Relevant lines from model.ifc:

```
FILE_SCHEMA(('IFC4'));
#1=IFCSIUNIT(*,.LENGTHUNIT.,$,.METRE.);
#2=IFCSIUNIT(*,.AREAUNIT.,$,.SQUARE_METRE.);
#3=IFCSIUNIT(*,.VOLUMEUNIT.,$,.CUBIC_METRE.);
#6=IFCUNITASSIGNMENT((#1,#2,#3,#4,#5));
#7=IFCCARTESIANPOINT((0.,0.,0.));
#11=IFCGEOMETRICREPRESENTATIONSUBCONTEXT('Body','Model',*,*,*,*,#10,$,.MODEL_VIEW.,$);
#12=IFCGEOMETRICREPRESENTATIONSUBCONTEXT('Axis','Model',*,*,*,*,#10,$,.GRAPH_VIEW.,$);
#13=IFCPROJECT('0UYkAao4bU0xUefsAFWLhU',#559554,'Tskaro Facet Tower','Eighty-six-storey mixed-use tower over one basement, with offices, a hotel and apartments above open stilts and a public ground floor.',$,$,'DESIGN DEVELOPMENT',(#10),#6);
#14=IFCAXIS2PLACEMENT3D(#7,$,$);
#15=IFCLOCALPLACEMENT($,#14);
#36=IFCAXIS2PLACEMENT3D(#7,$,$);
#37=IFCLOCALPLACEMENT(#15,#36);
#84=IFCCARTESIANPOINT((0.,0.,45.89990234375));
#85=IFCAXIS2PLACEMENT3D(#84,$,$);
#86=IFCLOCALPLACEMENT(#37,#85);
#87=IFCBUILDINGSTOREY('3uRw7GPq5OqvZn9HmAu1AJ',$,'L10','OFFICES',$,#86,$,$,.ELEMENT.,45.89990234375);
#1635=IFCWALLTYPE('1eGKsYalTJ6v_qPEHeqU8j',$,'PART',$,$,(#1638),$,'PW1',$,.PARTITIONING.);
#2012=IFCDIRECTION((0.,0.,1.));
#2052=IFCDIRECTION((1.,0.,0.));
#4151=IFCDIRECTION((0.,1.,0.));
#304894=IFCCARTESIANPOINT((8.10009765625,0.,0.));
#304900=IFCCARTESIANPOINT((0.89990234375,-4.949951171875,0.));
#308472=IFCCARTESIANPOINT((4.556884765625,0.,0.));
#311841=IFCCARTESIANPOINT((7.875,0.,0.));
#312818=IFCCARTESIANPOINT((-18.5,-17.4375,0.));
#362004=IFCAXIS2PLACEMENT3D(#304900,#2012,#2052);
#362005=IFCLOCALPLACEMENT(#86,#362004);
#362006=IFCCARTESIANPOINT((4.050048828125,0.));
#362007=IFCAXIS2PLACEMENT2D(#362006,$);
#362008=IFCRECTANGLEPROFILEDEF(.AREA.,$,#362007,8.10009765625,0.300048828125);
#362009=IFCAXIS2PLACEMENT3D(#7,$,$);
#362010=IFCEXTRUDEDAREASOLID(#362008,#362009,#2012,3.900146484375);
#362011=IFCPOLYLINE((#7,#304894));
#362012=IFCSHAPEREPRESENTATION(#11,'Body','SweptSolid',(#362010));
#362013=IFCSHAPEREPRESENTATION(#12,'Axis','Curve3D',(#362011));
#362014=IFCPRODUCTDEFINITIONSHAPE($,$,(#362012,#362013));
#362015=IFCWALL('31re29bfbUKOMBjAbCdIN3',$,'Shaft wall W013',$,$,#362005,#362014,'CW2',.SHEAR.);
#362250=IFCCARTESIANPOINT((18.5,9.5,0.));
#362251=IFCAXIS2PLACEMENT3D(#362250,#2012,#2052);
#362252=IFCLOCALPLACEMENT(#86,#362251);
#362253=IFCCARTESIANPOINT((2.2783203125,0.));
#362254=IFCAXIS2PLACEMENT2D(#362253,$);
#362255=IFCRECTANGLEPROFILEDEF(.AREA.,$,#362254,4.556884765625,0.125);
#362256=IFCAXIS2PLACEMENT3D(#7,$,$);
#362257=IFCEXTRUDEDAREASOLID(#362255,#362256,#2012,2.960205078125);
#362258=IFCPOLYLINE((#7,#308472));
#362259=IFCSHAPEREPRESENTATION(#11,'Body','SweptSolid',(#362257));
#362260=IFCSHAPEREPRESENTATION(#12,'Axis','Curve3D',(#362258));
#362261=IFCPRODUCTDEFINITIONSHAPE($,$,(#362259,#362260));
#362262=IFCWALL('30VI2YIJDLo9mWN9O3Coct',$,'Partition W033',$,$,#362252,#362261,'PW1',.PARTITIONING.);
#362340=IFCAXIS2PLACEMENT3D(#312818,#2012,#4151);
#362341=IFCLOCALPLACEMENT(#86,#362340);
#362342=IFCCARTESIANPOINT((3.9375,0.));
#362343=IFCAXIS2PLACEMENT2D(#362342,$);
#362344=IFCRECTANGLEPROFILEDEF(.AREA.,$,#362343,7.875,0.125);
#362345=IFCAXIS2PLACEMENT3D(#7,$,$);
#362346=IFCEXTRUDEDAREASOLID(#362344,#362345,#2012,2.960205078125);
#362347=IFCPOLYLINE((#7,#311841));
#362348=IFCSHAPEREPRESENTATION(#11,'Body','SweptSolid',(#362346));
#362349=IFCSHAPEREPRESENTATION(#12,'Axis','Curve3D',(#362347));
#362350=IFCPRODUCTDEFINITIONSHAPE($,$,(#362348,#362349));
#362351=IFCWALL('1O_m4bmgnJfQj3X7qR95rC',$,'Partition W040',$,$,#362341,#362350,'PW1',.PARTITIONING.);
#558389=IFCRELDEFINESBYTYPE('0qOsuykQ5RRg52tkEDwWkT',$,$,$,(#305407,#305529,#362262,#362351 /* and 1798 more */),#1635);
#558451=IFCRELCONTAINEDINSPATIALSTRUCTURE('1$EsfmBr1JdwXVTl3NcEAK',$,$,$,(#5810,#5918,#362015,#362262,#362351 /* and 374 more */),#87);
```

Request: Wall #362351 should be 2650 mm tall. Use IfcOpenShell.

```python
import ifcopenshell
import ifcopenshell.geom
import ifcopenshell.util.representation
import ifcopenshell.util.shape
import ifcopenshell.util.unit

model = ifcopenshell.open("model.ifc")
unit_scale = ifcopenshell.util.unit.calculate_unit_scale(model)
settings = ifcopenshell.geom.settings()


def volume(element):
    """Net volume in cubic metres, openings subtracted."""
    shape = ifcopenshell.geom.create_shape(settings, element)
    return ifcopenshell.util.shape.get_volume(shape.geometry)


wall = model.by_id(362351)
before = volume(wall)

body = ifcopenshell.util.representation.get_representation(wall, "Model", "Body")
solid = body.Items[0]
old_height = solid.Depth
solid.Depth = 2.65 / unit_scale
after = volume(wall)

print(f"height {old_height:g} -> {solid.Depth:g}, volume {before:.3f} -> {after:.3f} m3")

model.write("model_rev.ifc")
```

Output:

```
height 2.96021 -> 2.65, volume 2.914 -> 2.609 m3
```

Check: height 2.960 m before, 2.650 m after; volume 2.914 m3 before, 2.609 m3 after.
